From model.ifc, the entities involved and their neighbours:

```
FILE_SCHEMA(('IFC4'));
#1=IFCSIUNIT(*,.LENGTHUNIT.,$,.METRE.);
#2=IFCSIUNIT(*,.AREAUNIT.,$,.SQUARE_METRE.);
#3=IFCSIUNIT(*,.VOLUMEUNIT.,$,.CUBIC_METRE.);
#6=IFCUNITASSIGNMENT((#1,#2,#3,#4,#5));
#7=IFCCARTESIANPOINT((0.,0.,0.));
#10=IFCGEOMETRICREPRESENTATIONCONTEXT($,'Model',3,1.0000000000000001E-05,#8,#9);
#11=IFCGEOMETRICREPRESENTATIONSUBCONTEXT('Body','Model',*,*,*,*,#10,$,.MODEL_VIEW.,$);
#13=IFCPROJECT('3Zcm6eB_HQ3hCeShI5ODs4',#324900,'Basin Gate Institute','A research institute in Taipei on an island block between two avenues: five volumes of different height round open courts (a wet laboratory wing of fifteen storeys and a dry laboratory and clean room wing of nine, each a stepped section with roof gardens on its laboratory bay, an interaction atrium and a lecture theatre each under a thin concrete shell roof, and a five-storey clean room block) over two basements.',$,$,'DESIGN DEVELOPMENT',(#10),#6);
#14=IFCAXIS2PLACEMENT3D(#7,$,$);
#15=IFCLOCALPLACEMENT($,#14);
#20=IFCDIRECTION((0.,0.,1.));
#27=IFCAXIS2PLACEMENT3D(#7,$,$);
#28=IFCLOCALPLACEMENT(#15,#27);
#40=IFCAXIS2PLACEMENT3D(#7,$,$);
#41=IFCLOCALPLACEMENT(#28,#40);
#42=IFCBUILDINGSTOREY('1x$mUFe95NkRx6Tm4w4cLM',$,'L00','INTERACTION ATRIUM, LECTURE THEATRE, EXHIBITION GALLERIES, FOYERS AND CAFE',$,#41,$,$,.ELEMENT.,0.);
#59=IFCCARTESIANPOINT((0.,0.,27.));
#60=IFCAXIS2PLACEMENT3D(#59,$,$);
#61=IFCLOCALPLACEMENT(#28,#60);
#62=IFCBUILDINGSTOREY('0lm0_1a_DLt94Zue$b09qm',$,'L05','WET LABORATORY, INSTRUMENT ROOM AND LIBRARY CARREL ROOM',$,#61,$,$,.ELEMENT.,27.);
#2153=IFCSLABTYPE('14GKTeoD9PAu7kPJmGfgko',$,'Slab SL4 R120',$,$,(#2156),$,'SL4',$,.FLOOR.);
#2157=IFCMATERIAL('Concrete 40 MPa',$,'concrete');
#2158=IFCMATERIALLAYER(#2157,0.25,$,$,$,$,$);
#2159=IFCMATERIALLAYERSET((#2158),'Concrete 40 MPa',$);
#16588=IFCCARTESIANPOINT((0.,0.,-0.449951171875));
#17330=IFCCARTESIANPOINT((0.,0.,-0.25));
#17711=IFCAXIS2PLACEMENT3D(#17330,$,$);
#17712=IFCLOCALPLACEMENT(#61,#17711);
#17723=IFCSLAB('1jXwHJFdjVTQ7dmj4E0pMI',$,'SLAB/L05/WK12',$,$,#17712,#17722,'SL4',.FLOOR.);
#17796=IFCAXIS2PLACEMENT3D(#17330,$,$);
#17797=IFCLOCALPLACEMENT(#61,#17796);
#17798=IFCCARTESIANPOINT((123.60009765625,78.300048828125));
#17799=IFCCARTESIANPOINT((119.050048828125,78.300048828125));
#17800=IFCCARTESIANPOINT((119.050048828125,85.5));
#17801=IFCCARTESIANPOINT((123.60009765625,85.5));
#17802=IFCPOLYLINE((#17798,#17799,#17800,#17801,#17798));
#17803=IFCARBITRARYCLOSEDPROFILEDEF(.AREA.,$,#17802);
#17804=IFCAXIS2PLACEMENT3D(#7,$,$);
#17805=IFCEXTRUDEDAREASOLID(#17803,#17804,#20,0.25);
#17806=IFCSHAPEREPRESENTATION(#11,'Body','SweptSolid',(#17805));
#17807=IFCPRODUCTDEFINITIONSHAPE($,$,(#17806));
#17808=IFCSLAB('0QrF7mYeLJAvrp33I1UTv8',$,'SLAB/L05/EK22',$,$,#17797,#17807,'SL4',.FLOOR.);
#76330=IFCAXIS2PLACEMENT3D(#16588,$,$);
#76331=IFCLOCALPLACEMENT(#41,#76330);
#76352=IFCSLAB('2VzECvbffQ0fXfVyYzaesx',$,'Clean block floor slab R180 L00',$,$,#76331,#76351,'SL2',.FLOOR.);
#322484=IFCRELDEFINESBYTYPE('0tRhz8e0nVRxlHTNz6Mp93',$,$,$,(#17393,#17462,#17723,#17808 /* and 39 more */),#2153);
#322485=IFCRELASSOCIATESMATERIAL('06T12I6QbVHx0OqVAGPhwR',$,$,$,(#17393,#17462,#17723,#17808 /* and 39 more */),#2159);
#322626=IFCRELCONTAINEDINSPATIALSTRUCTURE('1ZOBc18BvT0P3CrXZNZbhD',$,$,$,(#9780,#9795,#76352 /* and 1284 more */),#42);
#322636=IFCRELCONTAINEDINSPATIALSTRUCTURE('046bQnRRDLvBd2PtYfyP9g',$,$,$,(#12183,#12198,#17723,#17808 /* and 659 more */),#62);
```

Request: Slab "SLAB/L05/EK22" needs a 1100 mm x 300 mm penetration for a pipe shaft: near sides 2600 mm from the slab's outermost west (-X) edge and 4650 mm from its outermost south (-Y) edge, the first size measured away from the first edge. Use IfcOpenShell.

```python
import numpy as np
import ifcopenshell
import ifcopenshell.api.feature
import ifcopenshell.api.geometry
import ifcopenshell.api.root
import ifcopenshell.geom
import ifcopenshell.util.placement
import ifcopenshell.util.representation
import ifcopenshell.util.shape
import ifcopenshell.util.unit

model = ifcopenshell.open("model.ifc")
unit_scale = ifcopenshell.util.unit.calculate_unit_scale(model)
settings = ifcopenshell.geom.settings()


def volume(element):
    """Net volume in cubic metres, openings subtracted."""
    shape = ifcopenshell.geom.create_shape(settings, element)
    return ifcopenshell.util.shape.get_volume(shape.geometry)


slab = model.by_guid("0QrF7mYeLJAvrp33I1UTv8")
before = volume(slab)

# Extent in the slab's own axes, in metres. The edges named are its -X and -Y sides.
slab_shape = ifcopenshell.geom.create_shape(settings, slab)
vertices = ifcopenshell.util.shape.get_vertices(slab_shape.geometry)
x_min, y_min, bottom = vertices.min(axis=0)
top = vertices[:, 2].max()

opening = ifcopenshell.api.root.create_entity(model, ifc_class="IfcOpeningElement", name="Pipe shaft opening", predefined_type="OPENING")
context = ifcopenshell.util.representation.get_context(model, "Model", "Body", "MODEL_VIEW")
width, depth = 1.1, 0.3
outline = [(0.0, 0.0), (width, 0.0), (width, depth), (0.0, depth), (0.0, 0.0)]
# Overshoot both faces by 50 mm so the cut is clean.
shape = ifcopenshell.api.geometry.add_slab_representation(
    model, context=context, depth=top - bottom + 0.1, polyline=outline
)
ifcopenshell.api.geometry.assign_representation(model, product=opening, representation=shape)

matrix = ifcopenshell.util.placement.get_local_placement(slab.ObjectPlacement)
matrix[:, 3] = matrix @ np.append(np.array([x_min + 2.6, y_min + 4.65, bottom - 0.05]) / unit_scale, 1.0)
ifcopenshell.api.geometry.edit_object_placement(model, product=opening, matrix=matrix, is_si=False)
ifcopenshell.api.feature.add_feature(model, feature=opening, element=slab)

after = volume(slab)

print(f"slab volume {before:.3f} -> {after:.3f} m3")

model.write("model_v2.ifc")
```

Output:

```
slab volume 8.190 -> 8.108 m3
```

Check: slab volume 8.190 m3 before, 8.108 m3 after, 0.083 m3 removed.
